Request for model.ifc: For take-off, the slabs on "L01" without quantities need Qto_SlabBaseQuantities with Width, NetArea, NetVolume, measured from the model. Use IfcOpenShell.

First a look at what the model holds.

```python
import ifcopenshell
import ifcopenshell.util.element
import ifcopenshell.util.unit

model = ifcopenshell.open("model.ifc")
print(model.schema)
for unit_type in ("LENGTHUNIT", "AREAUNIT", "VOLUMEUNIT"):
    print(unit_type, ifcopenshell.util.unit.calculate_unit_scale(model, unit_type))
storey = next(s for s in model.by_type("IfcBuildingStorey") if s.Name == "L01")
slabs = [e for e in ifcopenshell.util.element.get_decomposition(storey) if e.is_a("IfcSlab")]
for e in sorted(slabs, key=lambda e: e.id()):
    print(e.id(), e.is_a(), e.Name, list(ifcopenshell.util.element.get_psets(e, qtos_only=True)), sep=" | ")
```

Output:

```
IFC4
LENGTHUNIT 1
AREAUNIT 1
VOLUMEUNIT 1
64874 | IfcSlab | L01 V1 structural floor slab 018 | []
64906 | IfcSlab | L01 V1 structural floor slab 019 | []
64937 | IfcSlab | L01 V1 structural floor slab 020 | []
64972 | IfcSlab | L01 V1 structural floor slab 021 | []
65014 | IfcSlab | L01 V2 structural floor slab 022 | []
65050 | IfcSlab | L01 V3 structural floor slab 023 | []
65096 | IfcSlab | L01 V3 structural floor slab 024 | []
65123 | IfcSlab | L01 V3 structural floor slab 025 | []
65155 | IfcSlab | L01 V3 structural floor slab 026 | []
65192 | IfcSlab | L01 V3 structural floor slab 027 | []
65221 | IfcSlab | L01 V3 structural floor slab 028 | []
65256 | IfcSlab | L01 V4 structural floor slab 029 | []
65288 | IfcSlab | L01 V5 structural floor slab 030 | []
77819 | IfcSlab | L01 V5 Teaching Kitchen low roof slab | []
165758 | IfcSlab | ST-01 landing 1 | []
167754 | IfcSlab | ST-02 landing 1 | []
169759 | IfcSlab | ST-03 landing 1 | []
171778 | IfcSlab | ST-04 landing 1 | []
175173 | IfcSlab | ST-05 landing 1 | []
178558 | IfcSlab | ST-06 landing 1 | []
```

```python
import ifcopenshell
import ifcopenshell.api.pset
import ifcopenshell.geom
import ifcopenshell.util.element
import ifcopenshell.util.shape
import ifcopenshell.util.unit

model = ifcopenshell.open("model.ifc")
unit_scale = ifcopenshell.util.unit.calculate_unit_scale(model)
area_scale = ifcopenshell.util.unit.calculate_unit_scale(model, "AREAUNIT")
volume_scale = ifcopenshell.util.unit.calculate_unit_scale(model, "VOLUMEUNIT")
settings = ifcopenshell.geom.settings()

storey = next(s for s in model.by_type("IfcBuildingStorey") if s.Name == "L01")
slabs = [e for e in ifcopenshell.util.element.get_decomposition(storey) if e.is_a("IfcSlab")]

for e in sorted(slabs, key=lambda e: e.id()):
    if ifcopenshell.util.element.get_psets(e, qtos_only=True, should_inherit=False):
        continue
    # Geometry comes back in metres, in the element's own axes.
    shape = ifcopenshell.geom.create_shape(settings, e)
    values = {
        "Width": ifcopenshell.util.shape.get_z(shape.geometry) / unit_scale,
        "NetArea": ifcopenshell.util.shape.get_footprint_area(shape.geometry) / area_scale,
        "NetVolume": ifcopenshell.util.shape.get_volume(shape.geometry) / volume_scale,
    }
    qto = ifcopenshell.api.pset.add_qto(model, product=e, name="Qto_SlabBaseQuantities")
    ifcopenshell.api.pset.edit_qto(model, qto=qto, properties=values)
    print(e.id(), {k: round(v, 3) for k, v in values.items()})

model.write("model_rev.ifc")
```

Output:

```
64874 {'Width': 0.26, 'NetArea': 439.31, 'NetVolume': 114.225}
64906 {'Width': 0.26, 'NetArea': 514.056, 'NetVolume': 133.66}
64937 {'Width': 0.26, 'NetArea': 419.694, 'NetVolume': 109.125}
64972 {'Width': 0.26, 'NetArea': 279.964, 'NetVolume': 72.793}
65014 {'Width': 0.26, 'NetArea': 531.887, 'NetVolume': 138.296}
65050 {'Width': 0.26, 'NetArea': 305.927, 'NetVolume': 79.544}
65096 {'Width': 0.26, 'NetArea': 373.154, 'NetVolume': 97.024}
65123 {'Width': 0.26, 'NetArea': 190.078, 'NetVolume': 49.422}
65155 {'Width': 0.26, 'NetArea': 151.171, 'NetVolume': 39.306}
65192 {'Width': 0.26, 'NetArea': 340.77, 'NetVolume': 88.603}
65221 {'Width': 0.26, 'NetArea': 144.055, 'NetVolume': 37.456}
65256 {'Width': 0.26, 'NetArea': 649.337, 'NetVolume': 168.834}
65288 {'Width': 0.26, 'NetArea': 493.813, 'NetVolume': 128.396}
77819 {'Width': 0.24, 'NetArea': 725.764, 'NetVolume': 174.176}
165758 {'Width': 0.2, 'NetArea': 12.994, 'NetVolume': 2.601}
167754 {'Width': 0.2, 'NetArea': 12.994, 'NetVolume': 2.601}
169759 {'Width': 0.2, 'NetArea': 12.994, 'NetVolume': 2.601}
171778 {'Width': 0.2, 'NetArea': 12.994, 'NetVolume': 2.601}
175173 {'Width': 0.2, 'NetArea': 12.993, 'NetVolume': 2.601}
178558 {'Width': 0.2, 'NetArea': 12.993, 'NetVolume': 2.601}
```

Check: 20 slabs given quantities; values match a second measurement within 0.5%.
